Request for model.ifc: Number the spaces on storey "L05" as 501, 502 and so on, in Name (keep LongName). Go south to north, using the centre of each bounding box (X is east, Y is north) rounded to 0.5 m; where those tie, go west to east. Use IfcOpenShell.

First a look at what the model holds.

```python
import ifcopenshell
import ifcopenshell.util.element
import ifcopenshell.util.placement

model = ifcopenshell.open("model.ifc")
print(model.schema)
storey = next(s for s in model.by_type("IfcBuildingStorey") if s.Name == "L05")
spaces = [e for e in ifcopenshell.util.element.get_decomposition(storey) if e.is_a("IfcSpace")]
for e in sorted(spaces, key=lambda e: e.id()):
    origin = ifcopenshell.util.placement.get_local_placement(e.ObjectPlacement)[:3, 3]
    print(e.id(), e.Name, e.LongName, origin.round(2) + 0.0, sep=" | ")
```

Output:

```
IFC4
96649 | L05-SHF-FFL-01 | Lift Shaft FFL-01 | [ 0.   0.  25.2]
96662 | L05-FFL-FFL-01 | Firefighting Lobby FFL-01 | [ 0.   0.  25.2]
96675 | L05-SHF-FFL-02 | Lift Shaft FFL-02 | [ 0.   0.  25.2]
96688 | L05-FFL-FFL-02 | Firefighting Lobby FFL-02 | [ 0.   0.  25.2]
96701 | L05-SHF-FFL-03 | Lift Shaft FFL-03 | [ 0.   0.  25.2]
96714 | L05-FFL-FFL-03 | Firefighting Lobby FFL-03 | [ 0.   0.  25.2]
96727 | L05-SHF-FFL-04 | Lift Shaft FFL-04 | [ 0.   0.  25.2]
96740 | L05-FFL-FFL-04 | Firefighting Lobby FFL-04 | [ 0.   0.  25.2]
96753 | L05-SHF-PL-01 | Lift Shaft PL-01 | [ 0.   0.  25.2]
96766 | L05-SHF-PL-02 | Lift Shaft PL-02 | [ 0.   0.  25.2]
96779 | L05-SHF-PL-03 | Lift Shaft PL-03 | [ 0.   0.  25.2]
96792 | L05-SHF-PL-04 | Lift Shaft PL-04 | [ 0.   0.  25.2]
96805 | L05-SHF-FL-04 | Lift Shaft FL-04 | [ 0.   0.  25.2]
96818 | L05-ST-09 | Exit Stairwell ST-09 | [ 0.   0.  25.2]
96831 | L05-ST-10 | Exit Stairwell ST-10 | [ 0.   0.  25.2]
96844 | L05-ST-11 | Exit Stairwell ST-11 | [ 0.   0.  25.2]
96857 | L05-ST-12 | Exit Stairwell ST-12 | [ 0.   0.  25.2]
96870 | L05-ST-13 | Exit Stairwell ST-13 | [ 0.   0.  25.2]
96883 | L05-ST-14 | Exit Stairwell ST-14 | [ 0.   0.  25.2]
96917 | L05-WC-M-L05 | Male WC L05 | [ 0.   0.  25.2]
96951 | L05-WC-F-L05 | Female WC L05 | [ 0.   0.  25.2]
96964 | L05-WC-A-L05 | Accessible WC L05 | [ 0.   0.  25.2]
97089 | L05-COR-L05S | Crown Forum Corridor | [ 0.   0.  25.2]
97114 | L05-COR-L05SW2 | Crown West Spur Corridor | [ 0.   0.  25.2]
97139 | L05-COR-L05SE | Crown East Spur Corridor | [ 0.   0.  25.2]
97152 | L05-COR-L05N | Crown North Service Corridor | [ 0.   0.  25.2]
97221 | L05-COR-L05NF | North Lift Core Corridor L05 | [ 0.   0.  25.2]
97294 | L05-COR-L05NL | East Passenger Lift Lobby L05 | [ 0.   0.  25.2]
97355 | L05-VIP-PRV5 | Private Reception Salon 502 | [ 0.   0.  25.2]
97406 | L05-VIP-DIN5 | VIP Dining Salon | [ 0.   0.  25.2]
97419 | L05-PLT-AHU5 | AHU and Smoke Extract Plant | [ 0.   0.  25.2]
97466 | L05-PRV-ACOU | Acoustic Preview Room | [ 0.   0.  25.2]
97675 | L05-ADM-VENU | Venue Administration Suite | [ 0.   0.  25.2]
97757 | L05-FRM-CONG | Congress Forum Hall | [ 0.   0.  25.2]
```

```python
import ifcopenshell
import ifcopenshell.geom
import ifcopenshell.util.element
import ifcopenshell.util.shape

model = ifcopenshell.open("model.ifc")
settings = ifcopenshell.geom.settings()
settings.set("use-world-coords", True)


def centre(element):
    shape = ifcopenshell.geom.create_shape(settings, element)
    return ifcopenshell.util.shape.get_bbox_centroid(shape.geometry)


storey = next(s for s in model.by_type("IfcBuildingStorey") if s.Name == "L05")
spaces = [e for e in ifcopenshell.util.element.get_decomposition(storey) if e.is_a("IfcSpace")]

# Insertion points can sit at a corner or the storey origin, so sort by the geometry (in metres).
centres = {e: centre(e) for e in spaces}
spaces.sort(key=lambda e: (round(centres[e][1] / 0.5), centres[e][0]))

for i, e in enumerate(spaces, start=1):
    number = f"5{i:02d}"
    e.Name = number
    print(e.id(), number)

model.write("model_updated.ifc")
```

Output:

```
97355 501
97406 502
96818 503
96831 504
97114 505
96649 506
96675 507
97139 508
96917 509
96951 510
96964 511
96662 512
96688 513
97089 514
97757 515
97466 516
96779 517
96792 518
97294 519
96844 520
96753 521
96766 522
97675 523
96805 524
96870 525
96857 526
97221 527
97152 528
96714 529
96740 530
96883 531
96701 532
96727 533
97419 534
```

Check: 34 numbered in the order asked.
